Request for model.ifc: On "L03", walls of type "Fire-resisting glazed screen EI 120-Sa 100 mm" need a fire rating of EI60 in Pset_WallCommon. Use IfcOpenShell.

First a look at what the model holds.

```python
import ifcopenshell
import ifcopenshell.util.element

model = ifcopenshell.open("model.ifc")
print(model.schema)
storey = next(s for s in model.by_type("IfcBuildingStorey") if s.Name == "L03")
walls = [e for e in ifcopenshell.util.element.get_decomposition(storey) if e.is_a("IfcWall")]
seen = {}
for e in walls:
    element_type = ifcopenshell.util.element.get_type(e)
    key = (element_type.Name if element_type != e and element_type else None, ifcopenshell.util.element.get_pset(e, "Pset_WallCommon", "FireRating"))
    seen[key] = seen.get(key, 0) + 1
for (name, value), count in sorted(seen.items(), key=str):
    print(count, "x", name, "|", value)
```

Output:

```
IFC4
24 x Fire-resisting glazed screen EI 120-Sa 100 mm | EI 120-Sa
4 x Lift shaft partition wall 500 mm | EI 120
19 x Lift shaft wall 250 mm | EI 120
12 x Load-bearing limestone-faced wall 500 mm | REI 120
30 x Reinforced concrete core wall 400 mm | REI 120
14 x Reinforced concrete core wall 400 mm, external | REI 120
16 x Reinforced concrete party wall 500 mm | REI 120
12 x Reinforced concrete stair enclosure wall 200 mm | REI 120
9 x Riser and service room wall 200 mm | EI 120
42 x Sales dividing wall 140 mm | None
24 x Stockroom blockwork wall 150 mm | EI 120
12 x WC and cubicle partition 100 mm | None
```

```python
import ifcopenshell
import ifcopenshell.api.pset
import ifcopenshell.util.element

model = ifcopenshell.open("model.ifc")

storey = next(s for s in model.by_type("IfcBuildingStorey") if s.Name == "L03")
walls = [e for e in ifcopenshell.util.element.get_decomposition(storey) if e.is_a("IfcWall")]

count = 0
for e in walls:
    element_type = ifcopenshell.util.element.get_type(e)
    if element_type in (None, e) or element_type.Name != "Fire-resisting glazed screen EI 120-Sa 100 mm":
        continue
    # add_pset returns the element's existing set when there is one.
    pset = ifcopenshell.api.pset.add_pset(model, product=e, name="Pset_WallCommon")
    ifcopenshell.api.pset.edit_pset(model, pset=pset, properties={"FireRating": "EI60"})
    count += 1

print(count, "walls updated")

model.write("model_updated.ifc")
```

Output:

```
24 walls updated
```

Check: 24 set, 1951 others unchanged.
